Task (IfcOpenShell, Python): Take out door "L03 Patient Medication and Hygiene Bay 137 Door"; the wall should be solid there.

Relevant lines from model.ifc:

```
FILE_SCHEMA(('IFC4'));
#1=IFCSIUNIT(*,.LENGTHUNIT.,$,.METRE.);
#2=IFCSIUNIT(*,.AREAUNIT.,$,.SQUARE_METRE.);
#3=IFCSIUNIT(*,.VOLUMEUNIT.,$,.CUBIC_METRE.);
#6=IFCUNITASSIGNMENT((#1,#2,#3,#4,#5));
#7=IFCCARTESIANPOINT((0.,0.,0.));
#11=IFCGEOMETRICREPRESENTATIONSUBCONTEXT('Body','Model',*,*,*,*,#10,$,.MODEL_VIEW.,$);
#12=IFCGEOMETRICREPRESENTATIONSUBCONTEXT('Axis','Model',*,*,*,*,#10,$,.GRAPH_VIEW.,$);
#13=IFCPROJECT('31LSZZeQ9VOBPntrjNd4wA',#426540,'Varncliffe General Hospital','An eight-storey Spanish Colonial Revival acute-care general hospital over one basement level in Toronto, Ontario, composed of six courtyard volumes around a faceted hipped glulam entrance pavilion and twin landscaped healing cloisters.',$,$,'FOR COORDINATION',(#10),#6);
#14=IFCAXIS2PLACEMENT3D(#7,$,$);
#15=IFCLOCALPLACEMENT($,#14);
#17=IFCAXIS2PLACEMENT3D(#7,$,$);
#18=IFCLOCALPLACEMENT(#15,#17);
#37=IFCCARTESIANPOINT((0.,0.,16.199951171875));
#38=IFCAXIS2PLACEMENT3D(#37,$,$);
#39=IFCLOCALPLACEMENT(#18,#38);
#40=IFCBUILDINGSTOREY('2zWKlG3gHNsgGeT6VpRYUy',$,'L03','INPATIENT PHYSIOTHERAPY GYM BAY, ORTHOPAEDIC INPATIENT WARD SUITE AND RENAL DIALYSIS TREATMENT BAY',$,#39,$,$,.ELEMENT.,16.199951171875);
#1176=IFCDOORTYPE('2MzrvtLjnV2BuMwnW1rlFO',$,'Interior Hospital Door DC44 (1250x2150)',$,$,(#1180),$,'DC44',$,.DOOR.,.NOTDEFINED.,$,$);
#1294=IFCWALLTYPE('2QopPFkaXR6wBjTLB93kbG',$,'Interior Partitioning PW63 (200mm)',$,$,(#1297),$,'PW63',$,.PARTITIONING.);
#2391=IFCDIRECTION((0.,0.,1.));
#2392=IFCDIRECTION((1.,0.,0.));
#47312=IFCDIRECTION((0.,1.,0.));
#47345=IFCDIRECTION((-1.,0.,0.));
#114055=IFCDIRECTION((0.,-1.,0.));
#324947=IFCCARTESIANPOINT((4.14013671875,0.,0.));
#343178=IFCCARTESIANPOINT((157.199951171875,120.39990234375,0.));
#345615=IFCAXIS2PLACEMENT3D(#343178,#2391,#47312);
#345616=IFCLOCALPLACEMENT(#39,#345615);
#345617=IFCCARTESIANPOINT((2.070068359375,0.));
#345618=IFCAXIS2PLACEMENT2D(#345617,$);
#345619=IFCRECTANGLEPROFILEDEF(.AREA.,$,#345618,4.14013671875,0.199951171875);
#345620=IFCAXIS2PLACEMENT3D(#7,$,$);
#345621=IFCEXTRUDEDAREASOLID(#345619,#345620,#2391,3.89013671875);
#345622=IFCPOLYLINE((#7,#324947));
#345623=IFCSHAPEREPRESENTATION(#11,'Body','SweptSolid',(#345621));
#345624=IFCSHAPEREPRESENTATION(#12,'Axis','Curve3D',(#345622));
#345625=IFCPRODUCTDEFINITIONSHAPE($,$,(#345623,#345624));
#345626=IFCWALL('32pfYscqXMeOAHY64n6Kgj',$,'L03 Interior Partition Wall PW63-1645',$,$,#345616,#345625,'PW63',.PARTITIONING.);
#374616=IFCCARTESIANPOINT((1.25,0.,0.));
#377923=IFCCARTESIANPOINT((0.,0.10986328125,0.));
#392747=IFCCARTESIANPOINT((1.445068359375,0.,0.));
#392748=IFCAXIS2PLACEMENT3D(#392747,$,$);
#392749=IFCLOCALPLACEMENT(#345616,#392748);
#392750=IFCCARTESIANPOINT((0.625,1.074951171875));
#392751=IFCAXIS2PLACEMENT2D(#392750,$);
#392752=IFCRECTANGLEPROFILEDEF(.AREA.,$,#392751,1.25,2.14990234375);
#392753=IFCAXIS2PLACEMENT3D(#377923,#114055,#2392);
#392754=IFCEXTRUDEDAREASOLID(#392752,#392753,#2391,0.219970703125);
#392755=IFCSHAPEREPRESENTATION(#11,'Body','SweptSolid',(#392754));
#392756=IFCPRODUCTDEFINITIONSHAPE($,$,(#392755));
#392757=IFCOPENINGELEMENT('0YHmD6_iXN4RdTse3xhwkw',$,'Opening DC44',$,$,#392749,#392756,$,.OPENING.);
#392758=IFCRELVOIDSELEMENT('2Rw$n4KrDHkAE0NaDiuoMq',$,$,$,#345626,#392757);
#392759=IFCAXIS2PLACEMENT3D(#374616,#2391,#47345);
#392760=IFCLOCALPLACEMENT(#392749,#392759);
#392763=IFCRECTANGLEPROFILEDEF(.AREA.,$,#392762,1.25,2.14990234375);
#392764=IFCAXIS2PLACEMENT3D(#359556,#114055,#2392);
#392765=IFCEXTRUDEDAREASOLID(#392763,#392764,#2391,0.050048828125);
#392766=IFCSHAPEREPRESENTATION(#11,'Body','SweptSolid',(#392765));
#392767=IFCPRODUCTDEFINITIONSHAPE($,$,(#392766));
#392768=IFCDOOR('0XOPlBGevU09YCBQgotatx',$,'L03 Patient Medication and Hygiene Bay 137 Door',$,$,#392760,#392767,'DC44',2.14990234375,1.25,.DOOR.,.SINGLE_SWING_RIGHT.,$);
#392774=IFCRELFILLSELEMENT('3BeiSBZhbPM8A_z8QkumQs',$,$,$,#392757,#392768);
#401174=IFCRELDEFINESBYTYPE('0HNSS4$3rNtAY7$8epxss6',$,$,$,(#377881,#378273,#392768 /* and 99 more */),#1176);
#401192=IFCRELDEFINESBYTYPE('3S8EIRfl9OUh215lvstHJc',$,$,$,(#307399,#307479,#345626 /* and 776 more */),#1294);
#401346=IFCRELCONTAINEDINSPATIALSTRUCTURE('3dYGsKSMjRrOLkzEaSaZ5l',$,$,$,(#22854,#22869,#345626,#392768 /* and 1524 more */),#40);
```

```python
import ifcopenshell
import ifcopenshell.api.feature
import ifcopenshell.api.root
import ifcopenshell.geom
import ifcopenshell.util.shape

model = ifcopenshell.open("model.ifc")
settings = ifcopenshell.geom.settings()


def volume(element):
    """Net volume in cubic metres, openings subtracted."""
    shape = ifcopenshell.geom.create_shape(settings, element)
    return ifcopenshell.util.shape.get_volume(shape.geometry)


door = model.by_guid("0XOPlBGevU09YCBQgotatx")
opening = door.FillsVoids[0].RelatingOpeningElement
wall = opening.VoidsElements[0].RelatingBuildingElement
before = volume(wall)

ifcopenshell.api.root.remove_product(model, product=door)
ifcopenshell.api.feature.remove_feature(model, feature=opening)

after = volume(wall)

print(f"wall volume {before:.3f} -> {after:.3f} m3")

model.write("model_edited.ifc")
```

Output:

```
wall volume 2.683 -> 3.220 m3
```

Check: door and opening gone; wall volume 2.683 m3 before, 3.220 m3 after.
